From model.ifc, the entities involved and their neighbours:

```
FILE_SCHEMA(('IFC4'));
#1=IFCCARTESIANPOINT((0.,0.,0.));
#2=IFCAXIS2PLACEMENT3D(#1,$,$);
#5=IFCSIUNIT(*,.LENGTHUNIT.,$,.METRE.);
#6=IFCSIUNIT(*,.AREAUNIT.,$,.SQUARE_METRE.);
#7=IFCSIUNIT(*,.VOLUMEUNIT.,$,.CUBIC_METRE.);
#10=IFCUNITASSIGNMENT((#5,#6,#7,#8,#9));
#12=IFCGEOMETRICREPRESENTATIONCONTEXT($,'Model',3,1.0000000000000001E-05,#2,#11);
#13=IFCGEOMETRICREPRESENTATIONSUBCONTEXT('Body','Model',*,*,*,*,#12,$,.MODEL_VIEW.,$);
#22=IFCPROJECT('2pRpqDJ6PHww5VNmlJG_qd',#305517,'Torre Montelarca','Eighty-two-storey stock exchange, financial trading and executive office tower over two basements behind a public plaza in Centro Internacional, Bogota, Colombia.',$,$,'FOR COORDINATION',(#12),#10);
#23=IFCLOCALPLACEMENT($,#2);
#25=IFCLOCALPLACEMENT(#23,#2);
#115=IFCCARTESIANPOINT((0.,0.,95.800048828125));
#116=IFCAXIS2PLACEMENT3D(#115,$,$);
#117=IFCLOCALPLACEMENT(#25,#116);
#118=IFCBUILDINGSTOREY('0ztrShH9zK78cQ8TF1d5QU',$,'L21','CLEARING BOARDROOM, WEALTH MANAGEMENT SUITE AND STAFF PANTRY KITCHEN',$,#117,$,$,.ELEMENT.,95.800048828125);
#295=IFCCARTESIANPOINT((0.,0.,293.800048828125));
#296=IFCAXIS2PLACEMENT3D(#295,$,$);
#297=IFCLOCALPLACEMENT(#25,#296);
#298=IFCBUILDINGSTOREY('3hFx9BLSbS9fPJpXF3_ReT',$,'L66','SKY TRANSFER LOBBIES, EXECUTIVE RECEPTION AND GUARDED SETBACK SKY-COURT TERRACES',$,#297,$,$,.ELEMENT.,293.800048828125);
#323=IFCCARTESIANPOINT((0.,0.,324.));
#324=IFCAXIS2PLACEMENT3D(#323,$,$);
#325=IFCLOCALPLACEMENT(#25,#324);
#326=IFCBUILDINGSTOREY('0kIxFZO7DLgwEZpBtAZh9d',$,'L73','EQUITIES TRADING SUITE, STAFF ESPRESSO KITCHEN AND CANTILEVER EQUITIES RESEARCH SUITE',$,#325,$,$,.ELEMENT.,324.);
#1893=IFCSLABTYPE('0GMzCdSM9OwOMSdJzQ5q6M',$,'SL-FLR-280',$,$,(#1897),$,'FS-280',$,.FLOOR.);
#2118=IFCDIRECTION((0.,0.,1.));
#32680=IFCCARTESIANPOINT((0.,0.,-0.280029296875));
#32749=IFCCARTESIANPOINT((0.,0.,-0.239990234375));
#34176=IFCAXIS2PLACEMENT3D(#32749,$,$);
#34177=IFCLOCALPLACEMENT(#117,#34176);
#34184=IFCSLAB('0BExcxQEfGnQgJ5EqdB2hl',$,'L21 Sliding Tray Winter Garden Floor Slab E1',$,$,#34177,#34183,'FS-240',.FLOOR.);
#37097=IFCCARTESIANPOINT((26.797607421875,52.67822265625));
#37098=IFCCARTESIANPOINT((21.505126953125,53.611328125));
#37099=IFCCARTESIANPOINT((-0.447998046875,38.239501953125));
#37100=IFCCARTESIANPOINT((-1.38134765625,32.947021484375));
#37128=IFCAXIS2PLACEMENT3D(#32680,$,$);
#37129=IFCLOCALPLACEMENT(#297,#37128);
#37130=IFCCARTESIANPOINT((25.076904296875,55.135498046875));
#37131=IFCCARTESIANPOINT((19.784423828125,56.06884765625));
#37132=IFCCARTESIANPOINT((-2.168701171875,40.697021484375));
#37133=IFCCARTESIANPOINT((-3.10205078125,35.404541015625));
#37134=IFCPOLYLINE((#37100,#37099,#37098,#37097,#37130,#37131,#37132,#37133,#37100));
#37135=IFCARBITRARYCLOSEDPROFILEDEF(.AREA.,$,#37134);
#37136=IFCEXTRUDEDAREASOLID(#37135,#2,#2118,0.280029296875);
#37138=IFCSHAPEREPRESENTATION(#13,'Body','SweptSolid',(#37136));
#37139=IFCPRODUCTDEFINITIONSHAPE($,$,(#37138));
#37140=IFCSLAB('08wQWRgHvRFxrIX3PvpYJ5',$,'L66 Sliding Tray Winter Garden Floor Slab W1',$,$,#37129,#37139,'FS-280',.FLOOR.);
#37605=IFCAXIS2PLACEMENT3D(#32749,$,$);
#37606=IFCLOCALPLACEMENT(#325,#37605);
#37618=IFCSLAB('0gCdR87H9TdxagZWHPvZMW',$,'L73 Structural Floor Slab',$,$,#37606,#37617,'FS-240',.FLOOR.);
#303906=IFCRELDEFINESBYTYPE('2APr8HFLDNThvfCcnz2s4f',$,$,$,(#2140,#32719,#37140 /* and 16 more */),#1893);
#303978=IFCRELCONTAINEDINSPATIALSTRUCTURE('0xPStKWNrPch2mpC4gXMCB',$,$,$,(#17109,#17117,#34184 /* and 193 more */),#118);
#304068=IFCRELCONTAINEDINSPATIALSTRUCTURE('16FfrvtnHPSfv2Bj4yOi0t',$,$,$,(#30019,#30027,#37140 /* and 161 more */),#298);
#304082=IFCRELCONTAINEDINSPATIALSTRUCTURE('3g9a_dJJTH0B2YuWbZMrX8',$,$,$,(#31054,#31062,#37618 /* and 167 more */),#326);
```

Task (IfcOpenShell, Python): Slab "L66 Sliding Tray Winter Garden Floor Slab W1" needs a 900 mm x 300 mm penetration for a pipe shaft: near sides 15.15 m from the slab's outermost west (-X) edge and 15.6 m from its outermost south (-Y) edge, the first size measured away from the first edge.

```python
import numpy as np
import ifcopenshell
import ifcopenshell.api.feature
import ifcopenshell.api.geometry
import ifcopenshell.api.root
import ifcopenshell.geom
import ifcopenshell.util.placement
import ifcopenshell.util.representation
import ifcopenshell.util.shape
import ifcopenshell.util.unit

model = ifcopenshell.open("model.ifc")
unit_scale = ifcopenshell.util.unit.calculate_unit_scale(model)
settings = ifcopenshell.geom.settings()


def volume(element):
    """Net volume in cubic metres, openings subtracted."""
    shape = ifcopenshell.geom.create_shape(settings, element)
    return ifcopenshell.util.shape.get_volume(shape.geometry)


slab = model.by_guid("08wQWRgHvRFxrIX3PvpYJ5")
before = volume(slab)

# Extent in the slab's own axes, in metres. The edges named are its -X and -Y sides.
slab_shape = ifcopenshell.geom.create_shape(settings, slab)
vertices = ifcopenshell.util.shape.get_vertices(slab_shape.geometry)
x_min, y_min, bottom = vertices.min(axis=0)
top = vertices[:, 2].max()

opening = ifcopenshell.api.root.create_entity(model, ifc_class="IfcOpeningElement", name="Pipe shaft opening", predefined_type="OPENING")
context = ifcopenshell.util.representation.get_context(model, "Model", "Body", "MODEL_VIEW")
width, depth = 0.9, 0.3
outline = [(0.0, 0.0), (width, 0.0), (width, depth), (0.0, depth), (0.0, 0.0)]
# Overshoot both faces by 50 mm so the cut is clean.
shape = ifcopenshell.api.geometry.add_slab_representation(
    model, context=context, depth=top - bottom + 0.1, polyline=outline
)
ifcopenshell.api.geometry.assign_representation(model, product=opening, representation=shape)

matrix = ifcopenshell.util.placement.get_local_placement(slab.ObjectPlacement)
matrix[:, 3] = matrix @ np.append(np.array([x_min + 15.15, y_min + 15.6, bottom - 0.05]) / unit_scale, 1.0)
ifcopenshell.api.geometry.edit_object_placement(model, product=opening, matrix=matrix, is_si=False)
ifcopenshell.api.feature.add_feature(model, feature=opening, element=slab)

after = volume(slab)

print(f"slab volume {before:.3f} -> {after:.3f} m3")

model.write("model_v2.ifc")
```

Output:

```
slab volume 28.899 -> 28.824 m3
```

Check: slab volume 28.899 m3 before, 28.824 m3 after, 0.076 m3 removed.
